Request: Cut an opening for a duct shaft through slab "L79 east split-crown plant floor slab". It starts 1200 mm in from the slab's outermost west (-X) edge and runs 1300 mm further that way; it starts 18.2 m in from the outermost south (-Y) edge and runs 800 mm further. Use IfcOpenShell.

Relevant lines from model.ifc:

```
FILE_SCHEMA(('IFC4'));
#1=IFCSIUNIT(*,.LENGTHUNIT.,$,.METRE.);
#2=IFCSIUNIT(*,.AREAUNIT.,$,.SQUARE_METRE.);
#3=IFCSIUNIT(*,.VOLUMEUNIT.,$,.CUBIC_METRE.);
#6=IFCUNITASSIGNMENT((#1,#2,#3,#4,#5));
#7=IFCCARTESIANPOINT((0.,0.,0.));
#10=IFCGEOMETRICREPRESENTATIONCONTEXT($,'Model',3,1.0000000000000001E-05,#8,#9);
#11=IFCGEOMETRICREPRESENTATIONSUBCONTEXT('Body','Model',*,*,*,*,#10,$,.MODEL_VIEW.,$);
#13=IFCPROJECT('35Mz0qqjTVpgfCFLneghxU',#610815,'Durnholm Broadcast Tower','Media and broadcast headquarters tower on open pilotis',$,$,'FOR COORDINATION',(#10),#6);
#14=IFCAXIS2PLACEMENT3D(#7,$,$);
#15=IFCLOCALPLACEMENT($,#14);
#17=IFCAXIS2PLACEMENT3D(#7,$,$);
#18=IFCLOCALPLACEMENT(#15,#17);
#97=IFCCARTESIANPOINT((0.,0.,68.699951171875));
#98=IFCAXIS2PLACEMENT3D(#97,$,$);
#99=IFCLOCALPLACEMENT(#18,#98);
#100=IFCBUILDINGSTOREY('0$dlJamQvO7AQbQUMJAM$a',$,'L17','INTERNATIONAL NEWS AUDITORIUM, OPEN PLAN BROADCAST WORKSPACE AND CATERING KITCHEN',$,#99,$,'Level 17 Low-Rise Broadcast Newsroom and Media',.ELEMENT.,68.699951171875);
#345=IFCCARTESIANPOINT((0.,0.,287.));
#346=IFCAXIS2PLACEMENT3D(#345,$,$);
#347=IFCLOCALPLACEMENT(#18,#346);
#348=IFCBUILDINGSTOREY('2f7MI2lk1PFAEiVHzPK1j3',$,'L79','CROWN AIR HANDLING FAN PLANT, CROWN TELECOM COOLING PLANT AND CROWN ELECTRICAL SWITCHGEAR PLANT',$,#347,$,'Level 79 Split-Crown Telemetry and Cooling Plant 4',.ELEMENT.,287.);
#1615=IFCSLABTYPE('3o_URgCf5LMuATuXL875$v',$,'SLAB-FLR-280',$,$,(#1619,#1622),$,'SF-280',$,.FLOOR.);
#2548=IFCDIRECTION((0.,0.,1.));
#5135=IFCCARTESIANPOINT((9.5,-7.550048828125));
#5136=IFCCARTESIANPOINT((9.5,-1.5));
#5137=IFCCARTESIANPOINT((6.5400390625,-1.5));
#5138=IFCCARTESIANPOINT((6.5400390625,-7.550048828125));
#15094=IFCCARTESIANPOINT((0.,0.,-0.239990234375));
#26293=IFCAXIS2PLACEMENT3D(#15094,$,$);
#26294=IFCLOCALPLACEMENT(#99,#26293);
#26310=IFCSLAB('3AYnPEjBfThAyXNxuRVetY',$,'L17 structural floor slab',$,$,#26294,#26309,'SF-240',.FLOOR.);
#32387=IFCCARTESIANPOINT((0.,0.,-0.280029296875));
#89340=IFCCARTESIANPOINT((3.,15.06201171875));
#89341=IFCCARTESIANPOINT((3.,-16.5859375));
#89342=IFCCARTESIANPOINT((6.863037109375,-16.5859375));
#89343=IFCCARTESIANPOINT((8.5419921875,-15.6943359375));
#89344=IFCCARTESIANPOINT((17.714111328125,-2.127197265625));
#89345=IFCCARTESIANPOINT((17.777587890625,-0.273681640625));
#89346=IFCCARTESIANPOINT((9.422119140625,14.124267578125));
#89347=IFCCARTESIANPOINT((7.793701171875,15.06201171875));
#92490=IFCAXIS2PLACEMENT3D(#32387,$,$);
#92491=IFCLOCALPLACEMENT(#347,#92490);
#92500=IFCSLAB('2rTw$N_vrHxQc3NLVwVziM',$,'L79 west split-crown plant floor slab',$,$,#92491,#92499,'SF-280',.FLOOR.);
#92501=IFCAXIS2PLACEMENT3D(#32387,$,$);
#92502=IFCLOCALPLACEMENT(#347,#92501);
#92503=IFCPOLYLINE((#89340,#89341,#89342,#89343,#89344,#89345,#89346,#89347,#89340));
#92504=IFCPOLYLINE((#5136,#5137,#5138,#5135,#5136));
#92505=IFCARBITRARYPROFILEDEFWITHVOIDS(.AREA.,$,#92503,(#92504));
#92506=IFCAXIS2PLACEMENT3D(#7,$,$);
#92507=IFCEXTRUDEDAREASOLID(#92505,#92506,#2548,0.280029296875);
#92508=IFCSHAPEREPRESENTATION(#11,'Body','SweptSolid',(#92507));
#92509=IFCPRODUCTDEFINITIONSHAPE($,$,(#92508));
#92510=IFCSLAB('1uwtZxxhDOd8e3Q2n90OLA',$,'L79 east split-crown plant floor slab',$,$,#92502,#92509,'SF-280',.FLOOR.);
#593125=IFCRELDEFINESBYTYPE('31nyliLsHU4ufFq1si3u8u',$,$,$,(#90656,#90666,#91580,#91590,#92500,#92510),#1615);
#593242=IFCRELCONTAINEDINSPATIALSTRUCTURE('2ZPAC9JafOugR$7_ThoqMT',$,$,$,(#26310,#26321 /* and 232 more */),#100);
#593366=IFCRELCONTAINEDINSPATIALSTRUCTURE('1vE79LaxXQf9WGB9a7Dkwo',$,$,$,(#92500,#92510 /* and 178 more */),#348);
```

```python
import numpy as np
import ifcopenshell
import ifcopenshell.api.feature
import ifcopenshell.api.geometry
import ifcopenshell.api.root
import ifcopenshell.geom
import ifcopenshell.util.placement
import ifcopenshell.util.representation
import ifcopenshell.util.shape
import ifcopenshell.util.unit

model = ifcopenshell.open("model.ifc")
unit_scale = ifcopenshell.util.unit.calculate_unit_scale(model)
settings = ifcopenshell.geom.settings()


def volume(element):
    """Net volume in cubic metres, openings subtracted."""
    shape = ifcopenshell.geom.create_shape(settings, element)
    return ifcopenshell.util.shape.get_volume(shape.geometry)


slab = model.by_guid("1uwtZxxhDOd8e3Q2n90OLA")
before = volume(slab)

# Extent in the slab's own axes, in metres. The edges named are its -X and -Y sides.
slab_shape = ifcopenshell.geom.create_shape(settings, slab)
vertices = ifcopenshell.util.shape.get_vertices(slab_shape.geometry)
x_min, y_min, bottom = vertices.min(axis=0)
top = vertices[:, 2].max()

opening = ifcopenshell.api.root.create_entity(model, ifc_class="IfcOpeningElement", name="Duct shaft opening", predefined_type="OPENING")
context = ifcopenshell.util.representation.get_context(model, "Model", "Body", "MODEL_VIEW")
width, depth = 1.3, 0.8
outline = [(0.0, 0.0), (width, 0.0), (width, depth), (0.0, depth), (0.0, 0.0)]
# Overshoot both faces by 50 mm so the cut is clean.
shape = ifcopenshell.api.geometry.add_slab_representation(
    model, context=context, depth=top - bottom + 0.1, polyline=outline
)
ifcopenshell.api.geometry.assign_representation(model, product=opening, representation=shape)

matrix = ifcopenshell.util.placement.get_local_placement(slab.ObjectPlacement)
matrix[:, 3] = matrix @ np.append(np.array([x_min + 1.2, y_min + 18.2, bottom - 0.05]) / unit_scale, 1.0)
ifcopenshell.api.geometry.edit_object_placement(model, product=opening, matrix=matrix, is_si=False)
ifcopenshell.api.feature.add_feature(model, feature=opening, element=slab)

after = volume(slab)

print(f"slab volume {before:.3f} -> {after:.3f} m3")

model.write("model_edited.ifc")
```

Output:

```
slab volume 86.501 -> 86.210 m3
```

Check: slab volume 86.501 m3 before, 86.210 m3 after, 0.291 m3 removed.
